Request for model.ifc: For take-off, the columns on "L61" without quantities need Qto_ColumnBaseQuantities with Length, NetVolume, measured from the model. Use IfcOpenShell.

First a look at what the model holds.

```python
import ifcopenshell
import ifcopenshell.util.element
import ifcopenshell.util.unit

model = ifcopenshell.open("model.ifc")
print(model.schema)
for unit_type in ("LENGTHUNIT", "AREAUNIT", "VOLUMEUNIT"):
    print(unit_type, ifcopenshell.util.unit.calculate_unit_scale(model, unit_type))
storey = next(s for s in model.by_type("IfcBuildingStorey") if s.Name == "L61")
columns = [e for e in ifcopenshell.util.element.get_decomposition(storey) if e.is_a("IfcColumn")]
for e in sorted(columns, key=lambda e: e.id()):
    print(e.id(), e.is_a(), e.Name, list(ifcopenshell.util.element.get_psets(e, qtos_only=True)), sep=" | ")
```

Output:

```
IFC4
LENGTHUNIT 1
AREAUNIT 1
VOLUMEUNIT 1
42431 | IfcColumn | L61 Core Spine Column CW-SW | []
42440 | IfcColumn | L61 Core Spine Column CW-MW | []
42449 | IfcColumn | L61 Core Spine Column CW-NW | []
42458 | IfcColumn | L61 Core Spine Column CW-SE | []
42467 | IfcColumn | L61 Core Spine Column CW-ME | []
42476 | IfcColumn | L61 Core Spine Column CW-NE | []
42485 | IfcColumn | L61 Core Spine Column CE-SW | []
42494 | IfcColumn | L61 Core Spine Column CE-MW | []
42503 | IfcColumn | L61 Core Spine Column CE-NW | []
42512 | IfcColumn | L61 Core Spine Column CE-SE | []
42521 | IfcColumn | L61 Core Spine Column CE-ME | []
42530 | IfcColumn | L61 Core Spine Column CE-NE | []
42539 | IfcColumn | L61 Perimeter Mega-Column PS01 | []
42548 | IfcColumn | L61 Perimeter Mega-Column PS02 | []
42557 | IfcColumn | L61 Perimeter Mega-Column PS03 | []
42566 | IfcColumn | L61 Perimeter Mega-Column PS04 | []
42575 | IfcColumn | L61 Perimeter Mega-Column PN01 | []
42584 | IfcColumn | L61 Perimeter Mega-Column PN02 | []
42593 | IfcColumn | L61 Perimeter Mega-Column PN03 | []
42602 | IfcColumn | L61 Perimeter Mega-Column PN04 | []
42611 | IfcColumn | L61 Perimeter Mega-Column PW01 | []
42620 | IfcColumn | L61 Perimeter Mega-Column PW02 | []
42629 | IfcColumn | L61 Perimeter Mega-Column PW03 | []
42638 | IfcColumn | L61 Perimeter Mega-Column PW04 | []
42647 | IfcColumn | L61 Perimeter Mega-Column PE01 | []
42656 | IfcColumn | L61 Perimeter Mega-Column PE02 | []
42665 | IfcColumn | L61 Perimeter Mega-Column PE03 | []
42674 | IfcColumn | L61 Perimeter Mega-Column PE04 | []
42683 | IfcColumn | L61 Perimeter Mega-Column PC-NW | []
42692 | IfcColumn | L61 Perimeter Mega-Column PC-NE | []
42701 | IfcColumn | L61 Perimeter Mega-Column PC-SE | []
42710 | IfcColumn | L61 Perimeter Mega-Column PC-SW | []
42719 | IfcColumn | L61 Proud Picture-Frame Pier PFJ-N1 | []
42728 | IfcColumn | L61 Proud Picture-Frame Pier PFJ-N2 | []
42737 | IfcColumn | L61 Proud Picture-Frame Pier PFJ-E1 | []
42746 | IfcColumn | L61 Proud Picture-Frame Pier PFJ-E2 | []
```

```python
import ifcopenshell
import ifcopenshell.api.pset
import ifcopenshell.geom
import ifcopenshell.util.element
import ifcopenshell.util.shape
import ifcopenshell.util.unit

model = ifcopenshell.open("model.ifc")
unit_scale = ifcopenshell.util.unit.calculate_unit_scale(model)
volume_scale = ifcopenshell.util.unit.calculate_unit_scale(model, "VOLUMEUNIT")
settings = ifcopenshell.geom.settings()

storey = next(s for s in model.by_type("IfcBuildingStorey") if s.Name == "L61")
columns = [e for e in ifcopenshell.util.element.get_decomposition(storey) if e.is_a("IfcColumn")]

for e in sorted(columns, key=lambda e: e.id()):
    if ifcopenshell.util.element.get_psets(e, qtos_only=True, should_inherit=False):
        continue
    # Geometry comes back in metres, in the element's own axes.
    shape = ifcopenshell.geom.create_shape(settings, e)
    values = {
        "Length": ifcopenshell.util.shape.get_z(shape.geometry) / unit_scale,
        "NetVolume": ifcopenshell.util.shape.get_volume(shape.geometry) / volume_scale,
    }
    qto = ifcopenshell.api.pset.add_qto(model, product=e, name="Qto_ColumnBaseQuantities")
    ifcopenshell.api.pset.edit_qto(model, qto=qto, properties=values)
    print(e.id(), {k: round(v, 3) for k, v in values.items()})

model.write("model_rev.ifc")
```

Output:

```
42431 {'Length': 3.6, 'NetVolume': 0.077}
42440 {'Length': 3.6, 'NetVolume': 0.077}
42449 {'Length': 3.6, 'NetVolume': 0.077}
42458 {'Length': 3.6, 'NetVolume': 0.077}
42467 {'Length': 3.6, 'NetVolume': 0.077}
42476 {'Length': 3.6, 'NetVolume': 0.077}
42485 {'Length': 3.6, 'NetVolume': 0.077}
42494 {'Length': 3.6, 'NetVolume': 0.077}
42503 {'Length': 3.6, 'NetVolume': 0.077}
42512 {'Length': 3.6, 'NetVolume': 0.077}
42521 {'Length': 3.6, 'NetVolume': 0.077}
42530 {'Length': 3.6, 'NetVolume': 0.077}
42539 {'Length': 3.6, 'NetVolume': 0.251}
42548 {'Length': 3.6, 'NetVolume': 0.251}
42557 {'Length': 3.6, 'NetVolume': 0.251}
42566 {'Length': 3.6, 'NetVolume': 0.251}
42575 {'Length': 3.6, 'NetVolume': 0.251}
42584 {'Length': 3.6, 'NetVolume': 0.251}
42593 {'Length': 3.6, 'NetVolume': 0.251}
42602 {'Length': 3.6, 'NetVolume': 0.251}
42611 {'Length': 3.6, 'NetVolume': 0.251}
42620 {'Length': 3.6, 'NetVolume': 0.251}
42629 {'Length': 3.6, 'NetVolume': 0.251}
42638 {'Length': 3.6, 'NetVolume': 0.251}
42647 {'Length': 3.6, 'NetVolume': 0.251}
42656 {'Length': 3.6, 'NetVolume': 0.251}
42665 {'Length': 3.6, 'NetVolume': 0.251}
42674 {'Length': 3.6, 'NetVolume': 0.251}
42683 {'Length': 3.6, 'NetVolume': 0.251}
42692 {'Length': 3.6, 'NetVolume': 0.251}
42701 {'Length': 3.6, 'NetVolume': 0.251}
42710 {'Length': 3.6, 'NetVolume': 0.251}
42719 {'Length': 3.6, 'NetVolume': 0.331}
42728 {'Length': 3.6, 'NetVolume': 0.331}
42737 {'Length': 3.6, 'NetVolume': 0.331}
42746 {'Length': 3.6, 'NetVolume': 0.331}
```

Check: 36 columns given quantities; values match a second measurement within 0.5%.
